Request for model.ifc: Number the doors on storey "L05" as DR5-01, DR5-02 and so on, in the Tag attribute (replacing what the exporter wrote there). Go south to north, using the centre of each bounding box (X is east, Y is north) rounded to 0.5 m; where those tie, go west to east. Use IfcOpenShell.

First a look at what the model holds.

```python
import ifcopenshell
import ifcopenshell.util.element
import ifcopenshell.util.placement

model = ifcopenshell.open("model.ifc")
print(model.schema)
storey = next(s for s in model.by_type("IfcBuildingStorey") if s.Name == "L05")
doors = [e for e in ifcopenshell.util.element.get_decomposition(storey) if e.is_a("IfcDoor")]
for e in sorted(doors, key=lambda e: e.id()):
    origin = ifcopenshell.util.placement.get_local_placement(e.ObjectPlacement)[:3, 3]
    print(e.id(), e.Tag, e.Name, origin.round(2) + 0.0, sep=" | ")
```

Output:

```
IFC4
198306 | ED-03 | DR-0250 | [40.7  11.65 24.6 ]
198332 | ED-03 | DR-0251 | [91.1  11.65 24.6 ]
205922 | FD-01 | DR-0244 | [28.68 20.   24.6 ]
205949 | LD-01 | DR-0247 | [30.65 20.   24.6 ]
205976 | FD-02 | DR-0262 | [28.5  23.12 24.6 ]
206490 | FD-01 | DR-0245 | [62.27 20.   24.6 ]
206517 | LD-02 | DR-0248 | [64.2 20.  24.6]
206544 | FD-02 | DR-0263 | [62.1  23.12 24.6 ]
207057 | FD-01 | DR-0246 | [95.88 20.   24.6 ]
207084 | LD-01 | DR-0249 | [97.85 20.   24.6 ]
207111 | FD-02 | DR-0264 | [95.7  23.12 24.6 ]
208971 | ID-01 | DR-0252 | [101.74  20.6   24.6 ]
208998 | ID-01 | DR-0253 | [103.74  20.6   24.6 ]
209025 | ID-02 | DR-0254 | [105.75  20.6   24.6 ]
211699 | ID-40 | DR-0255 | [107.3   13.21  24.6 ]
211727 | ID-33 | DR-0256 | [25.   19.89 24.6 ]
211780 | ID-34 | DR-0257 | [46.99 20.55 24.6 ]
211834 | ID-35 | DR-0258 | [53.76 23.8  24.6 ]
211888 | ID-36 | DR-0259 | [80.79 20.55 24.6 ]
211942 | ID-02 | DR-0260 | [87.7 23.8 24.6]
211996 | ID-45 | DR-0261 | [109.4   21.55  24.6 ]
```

```python
import ifcopenshell
import ifcopenshell.geom
import ifcopenshell.util.element
import ifcopenshell.util.shape

model = ifcopenshell.open("model.ifc")
settings = ifcopenshell.geom.settings()
settings.set("use-world-coords", True)


def centre(element):
    shape = ifcopenshell.geom.create_shape(settings, element)
    return ifcopenshell.util.shape.get_bbox_centroid(shape.geometry)


storey = next(s for s in model.by_type("IfcBuildingStorey") if s.Name == "L05")
doors = [e for e in ifcopenshell.util.element.get_decomposition(storey) if e.is_a("IfcDoor")]

# Insertion points can sit at a corner or the storey origin, so sort by the geometry (in metres).
centres = {e: centre(e) for e in doors}
doors.sort(key=lambda e: (round(centres[e][1] / 0.5), centres[e][0]))

for i, e in enumerate(doors, start=1):
    number = f"DR5-{i:02d}"
    e.Tag = number
    print(e.id(), number)

model.write("model_v2.ifc")
```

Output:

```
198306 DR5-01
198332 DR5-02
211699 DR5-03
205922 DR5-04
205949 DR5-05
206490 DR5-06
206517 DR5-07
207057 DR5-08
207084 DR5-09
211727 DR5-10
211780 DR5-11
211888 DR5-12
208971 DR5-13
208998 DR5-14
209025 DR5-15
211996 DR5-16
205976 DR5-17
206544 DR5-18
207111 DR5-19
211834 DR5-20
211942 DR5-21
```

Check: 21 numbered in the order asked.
